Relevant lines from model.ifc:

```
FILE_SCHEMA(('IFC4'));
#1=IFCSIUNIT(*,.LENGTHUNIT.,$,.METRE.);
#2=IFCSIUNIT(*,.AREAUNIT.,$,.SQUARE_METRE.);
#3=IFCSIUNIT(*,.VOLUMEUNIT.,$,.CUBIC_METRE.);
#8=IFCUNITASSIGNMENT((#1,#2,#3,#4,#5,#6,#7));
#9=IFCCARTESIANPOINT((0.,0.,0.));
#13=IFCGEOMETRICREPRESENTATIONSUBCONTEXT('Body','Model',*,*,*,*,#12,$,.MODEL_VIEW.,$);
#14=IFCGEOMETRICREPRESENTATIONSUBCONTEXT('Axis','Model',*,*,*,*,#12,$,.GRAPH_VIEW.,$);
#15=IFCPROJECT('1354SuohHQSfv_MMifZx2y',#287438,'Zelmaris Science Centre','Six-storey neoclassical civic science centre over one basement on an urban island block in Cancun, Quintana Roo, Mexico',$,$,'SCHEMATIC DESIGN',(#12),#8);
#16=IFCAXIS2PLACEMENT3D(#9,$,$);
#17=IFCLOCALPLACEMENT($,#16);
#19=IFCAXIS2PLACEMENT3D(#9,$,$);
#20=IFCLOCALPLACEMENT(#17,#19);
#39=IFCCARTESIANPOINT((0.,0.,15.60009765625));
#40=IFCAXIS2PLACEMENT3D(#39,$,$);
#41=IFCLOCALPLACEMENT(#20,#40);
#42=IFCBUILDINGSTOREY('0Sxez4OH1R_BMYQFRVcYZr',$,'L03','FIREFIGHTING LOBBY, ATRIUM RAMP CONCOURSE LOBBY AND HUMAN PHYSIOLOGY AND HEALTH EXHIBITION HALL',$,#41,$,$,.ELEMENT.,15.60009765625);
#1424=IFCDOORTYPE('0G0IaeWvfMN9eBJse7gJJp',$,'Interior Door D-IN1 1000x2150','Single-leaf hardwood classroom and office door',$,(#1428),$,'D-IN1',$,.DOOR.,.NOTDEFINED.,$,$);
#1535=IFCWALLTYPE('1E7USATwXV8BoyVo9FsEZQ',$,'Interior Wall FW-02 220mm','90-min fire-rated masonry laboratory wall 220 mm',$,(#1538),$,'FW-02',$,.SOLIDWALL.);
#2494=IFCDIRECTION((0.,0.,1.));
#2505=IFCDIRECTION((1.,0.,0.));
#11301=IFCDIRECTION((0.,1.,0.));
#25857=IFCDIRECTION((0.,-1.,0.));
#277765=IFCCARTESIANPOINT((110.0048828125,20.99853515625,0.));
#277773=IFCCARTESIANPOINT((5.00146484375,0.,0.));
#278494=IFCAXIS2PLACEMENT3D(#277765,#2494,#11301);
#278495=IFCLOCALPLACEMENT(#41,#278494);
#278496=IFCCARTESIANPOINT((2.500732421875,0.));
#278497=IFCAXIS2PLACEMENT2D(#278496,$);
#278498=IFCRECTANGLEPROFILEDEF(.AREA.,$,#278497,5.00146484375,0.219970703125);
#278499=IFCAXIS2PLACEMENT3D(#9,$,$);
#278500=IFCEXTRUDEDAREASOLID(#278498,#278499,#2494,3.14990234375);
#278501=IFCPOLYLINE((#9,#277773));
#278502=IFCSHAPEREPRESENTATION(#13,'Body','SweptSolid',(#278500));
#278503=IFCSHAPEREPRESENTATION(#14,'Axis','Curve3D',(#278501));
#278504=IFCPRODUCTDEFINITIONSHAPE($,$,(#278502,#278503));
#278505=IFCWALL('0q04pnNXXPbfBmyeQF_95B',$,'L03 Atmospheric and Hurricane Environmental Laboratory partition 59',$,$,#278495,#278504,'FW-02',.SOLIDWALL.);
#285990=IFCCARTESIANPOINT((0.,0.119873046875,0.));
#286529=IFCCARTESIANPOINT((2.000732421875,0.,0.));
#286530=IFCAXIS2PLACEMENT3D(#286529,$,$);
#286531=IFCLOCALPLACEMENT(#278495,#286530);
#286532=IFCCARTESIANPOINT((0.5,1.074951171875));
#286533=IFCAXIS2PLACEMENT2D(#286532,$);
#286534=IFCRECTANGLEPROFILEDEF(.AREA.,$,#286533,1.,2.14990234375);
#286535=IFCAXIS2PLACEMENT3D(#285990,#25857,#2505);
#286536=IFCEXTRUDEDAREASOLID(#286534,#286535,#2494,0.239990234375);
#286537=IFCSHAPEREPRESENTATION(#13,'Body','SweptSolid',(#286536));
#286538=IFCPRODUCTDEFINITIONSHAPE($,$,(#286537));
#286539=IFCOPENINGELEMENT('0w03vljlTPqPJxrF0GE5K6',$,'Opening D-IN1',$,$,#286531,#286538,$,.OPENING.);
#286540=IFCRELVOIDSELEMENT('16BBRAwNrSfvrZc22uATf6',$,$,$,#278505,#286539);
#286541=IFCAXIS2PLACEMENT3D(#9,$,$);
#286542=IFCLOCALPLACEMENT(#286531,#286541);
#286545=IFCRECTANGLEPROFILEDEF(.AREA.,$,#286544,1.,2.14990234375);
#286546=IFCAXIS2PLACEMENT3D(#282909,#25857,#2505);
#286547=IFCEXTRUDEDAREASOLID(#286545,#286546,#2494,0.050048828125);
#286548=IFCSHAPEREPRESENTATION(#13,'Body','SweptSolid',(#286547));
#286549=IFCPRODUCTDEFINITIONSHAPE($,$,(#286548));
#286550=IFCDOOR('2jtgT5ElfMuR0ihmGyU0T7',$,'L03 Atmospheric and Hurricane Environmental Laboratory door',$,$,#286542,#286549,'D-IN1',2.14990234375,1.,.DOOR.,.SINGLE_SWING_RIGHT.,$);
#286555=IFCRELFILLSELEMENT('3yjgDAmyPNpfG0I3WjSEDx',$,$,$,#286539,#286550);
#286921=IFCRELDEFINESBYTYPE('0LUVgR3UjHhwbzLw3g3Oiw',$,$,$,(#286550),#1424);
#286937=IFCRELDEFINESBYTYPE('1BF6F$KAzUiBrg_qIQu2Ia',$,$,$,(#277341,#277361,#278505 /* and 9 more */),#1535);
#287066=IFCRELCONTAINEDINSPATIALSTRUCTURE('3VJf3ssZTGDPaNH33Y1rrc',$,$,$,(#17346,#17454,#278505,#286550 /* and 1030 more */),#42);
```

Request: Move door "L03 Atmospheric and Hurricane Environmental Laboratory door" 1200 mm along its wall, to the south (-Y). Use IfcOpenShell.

```python
import ifcopenshell
import ifcopenshell.api.geometry
import ifcopenshell.util.placement
import ifcopenshell.util.unit

model = ifcopenshell.open("model.ifc")
unit_scale = ifcopenshell.util.unit.calculate_unit_scale(model)

door = model.by_guid("2jtgT5ElfMuR0ihmGyU0T7")
opening = door.FillsVoids[0].RelatingOpeningElement
wall = opening.VoidsElements[0].RelatingBuildingElement

wall_matrix = ifcopenshell.util.placement.get_local_placement(wall.ObjectPlacement)
shift = wall_matrix[:3, 0] * -1.2 / unit_scale
before = ifcopenshell.util.placement.get_local_placement(door.ObjectPlacement)[:3, 3].copy()

# The door is placed relative to its opening, so it follows when the opening moves.
matrix = ifcopenshell.util.placement.get_local_placement(opening.ObjectPlacement)
matrix[:3, 3] += shift
ifcopenshell.api.geometry.edit_object_placement(
    model, product=opening, matrix=matrix, is_si=False, should_transform_children=True
)

after = ifcopenshell.util.placement.get_local_placement(door.ObjectPlacement)[:3, 3]
print("door moved by", (after - before).round(3) + 0.0)

model.write("model_rev.ifc")
```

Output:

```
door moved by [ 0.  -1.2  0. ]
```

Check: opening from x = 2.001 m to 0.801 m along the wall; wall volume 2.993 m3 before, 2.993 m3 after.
